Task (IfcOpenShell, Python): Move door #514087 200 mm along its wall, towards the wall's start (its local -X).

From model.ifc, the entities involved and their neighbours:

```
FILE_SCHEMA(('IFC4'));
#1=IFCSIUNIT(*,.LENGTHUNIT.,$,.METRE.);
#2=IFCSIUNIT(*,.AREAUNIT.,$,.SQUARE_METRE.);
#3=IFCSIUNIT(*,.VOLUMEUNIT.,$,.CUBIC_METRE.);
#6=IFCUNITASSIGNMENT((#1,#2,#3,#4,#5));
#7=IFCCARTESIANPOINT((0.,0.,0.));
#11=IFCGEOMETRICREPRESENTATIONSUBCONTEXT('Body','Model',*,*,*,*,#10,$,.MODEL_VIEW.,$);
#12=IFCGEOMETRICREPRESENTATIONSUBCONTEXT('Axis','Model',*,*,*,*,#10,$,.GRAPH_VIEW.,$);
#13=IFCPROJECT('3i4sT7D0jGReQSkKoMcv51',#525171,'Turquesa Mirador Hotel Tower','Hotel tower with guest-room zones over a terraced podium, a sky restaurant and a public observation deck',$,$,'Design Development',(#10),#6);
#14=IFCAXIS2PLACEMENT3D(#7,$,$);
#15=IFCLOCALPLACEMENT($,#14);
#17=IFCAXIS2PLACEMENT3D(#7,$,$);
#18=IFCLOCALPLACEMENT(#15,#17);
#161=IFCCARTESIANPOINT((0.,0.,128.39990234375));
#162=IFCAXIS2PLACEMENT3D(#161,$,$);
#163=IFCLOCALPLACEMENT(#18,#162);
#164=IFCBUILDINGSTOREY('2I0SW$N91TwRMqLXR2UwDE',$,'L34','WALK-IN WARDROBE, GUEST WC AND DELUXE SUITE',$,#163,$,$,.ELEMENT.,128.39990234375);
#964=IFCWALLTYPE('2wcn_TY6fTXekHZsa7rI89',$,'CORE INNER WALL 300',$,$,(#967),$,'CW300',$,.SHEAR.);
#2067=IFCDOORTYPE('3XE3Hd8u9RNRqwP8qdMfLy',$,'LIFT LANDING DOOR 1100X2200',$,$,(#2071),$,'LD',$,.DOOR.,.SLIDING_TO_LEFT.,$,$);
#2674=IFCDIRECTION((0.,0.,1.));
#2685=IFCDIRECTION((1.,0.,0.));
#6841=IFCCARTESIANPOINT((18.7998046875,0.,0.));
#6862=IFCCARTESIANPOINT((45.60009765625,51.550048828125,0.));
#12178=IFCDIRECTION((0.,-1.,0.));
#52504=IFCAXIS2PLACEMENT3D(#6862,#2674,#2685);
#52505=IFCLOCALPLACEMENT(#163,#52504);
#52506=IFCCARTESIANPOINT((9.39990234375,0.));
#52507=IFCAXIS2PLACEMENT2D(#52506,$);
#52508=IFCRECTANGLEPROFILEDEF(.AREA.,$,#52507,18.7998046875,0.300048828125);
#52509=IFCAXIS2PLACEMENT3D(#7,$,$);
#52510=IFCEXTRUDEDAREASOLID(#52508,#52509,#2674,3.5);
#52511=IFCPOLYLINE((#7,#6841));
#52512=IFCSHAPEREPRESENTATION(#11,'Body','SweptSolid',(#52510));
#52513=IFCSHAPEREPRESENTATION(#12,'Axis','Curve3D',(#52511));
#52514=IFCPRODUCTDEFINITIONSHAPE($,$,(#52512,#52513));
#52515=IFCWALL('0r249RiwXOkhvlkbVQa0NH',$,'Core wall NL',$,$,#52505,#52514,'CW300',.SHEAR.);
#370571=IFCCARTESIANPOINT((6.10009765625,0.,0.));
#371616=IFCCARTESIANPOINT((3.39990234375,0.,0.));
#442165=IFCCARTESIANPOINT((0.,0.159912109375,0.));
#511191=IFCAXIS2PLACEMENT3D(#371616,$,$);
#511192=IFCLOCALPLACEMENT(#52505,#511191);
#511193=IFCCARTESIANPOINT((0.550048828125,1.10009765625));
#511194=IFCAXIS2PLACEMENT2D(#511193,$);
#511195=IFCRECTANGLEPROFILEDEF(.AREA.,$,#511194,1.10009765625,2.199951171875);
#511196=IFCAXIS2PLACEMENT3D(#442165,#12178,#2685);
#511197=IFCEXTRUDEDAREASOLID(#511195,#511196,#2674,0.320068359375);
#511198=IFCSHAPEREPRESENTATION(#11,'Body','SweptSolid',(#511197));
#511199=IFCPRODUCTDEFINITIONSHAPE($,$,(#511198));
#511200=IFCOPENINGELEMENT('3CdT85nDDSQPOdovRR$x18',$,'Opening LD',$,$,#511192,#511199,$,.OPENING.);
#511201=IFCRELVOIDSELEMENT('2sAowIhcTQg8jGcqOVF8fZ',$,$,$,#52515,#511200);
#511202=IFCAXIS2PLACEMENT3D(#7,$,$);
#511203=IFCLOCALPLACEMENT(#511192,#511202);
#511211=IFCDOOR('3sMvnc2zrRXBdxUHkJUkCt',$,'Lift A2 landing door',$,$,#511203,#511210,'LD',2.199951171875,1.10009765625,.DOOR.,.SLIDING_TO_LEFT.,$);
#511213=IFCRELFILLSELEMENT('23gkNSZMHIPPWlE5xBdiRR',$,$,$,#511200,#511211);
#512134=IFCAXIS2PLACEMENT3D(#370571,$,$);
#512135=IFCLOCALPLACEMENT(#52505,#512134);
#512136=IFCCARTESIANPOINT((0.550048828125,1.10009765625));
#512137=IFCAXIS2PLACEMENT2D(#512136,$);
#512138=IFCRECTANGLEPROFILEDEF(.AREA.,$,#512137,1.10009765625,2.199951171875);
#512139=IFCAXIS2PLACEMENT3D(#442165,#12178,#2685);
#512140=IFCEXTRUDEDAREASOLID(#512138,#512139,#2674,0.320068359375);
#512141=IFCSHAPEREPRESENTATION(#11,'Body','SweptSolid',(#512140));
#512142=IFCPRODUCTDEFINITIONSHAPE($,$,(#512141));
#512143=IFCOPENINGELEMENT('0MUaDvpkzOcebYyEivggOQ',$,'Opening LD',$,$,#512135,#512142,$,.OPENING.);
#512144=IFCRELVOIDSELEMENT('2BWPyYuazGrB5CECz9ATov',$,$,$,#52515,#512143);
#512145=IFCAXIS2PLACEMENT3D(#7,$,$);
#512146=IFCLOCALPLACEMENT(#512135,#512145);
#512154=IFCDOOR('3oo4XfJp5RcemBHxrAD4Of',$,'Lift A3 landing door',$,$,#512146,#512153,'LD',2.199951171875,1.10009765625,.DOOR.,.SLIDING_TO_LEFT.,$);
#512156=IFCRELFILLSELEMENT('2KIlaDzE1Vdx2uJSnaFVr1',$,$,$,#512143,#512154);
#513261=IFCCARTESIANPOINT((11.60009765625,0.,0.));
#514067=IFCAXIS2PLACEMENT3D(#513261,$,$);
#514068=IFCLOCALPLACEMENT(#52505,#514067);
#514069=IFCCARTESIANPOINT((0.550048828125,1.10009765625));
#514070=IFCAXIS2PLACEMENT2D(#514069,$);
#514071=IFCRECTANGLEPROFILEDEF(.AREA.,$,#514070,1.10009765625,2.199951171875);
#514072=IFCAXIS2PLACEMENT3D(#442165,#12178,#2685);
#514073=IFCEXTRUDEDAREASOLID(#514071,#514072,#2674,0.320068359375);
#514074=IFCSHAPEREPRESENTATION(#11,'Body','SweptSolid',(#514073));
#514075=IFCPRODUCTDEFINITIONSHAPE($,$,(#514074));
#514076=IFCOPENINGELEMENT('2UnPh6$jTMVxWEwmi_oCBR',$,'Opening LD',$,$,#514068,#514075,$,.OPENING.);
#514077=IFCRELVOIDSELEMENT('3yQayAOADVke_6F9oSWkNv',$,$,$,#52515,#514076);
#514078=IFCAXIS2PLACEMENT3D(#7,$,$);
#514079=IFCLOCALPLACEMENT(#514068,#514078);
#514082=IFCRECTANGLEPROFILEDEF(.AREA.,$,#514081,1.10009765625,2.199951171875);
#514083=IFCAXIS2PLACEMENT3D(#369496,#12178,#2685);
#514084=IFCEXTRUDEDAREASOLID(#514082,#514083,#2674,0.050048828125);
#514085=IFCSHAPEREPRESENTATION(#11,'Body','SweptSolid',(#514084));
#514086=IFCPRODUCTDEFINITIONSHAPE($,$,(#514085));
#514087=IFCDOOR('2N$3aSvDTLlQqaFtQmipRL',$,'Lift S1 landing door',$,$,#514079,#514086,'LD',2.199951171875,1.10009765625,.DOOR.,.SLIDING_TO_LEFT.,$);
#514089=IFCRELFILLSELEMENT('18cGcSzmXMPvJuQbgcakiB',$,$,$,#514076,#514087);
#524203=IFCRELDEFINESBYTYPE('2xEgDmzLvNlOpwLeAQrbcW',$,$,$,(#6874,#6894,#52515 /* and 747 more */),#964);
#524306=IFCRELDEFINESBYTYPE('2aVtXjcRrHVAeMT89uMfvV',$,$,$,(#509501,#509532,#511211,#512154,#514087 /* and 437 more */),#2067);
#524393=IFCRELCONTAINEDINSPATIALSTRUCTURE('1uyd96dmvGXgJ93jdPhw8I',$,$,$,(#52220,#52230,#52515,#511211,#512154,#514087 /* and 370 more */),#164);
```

```python
import ifcopenshell
import ifcopenshell.api.geometry
import ifcopenshell.util.placement

model = ifcopenshell.open("model.ifc")

door = model.by_id(514087)
opening = door.FillsVoids[0].RelatingOpeningElement
wall = opening.VoidsElements[0].RelatingBuildingElement

wall_matrix = ifcopenshell.util.placement.get_local_placement(wall.ObjectPlacement)
shift = wall_matrix[:3, 0] * -0.2
before = ifcopenshell.util.placement.get_local_placement(door.ObjectPlacement)[:3, 3].copy()

# The door is placed relative to its opening, so it follows when the opening moves.
matrix = ifcopenshell.util.placement.get_local_placement(opening.ObjectPlacement)
matrix[:3, 3] += shift
ifcopenshell.api.geometry.edit_object_placement(
    model, product=opening, matrix=matrix, is_si=False, should_transform_children=True
)

after = ifcopenshell.util.placement.get_local_placement(door.ObjectPlacement)[:3, 3]
print("door moved by", (after - before).round(3) + 0.0)

model.write("model-out.ifc")
```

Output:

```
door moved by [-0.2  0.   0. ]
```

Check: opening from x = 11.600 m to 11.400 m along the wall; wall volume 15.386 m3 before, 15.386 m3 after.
